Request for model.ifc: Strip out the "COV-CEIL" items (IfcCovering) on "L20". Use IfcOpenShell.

First a look at what the model holds.

```python
import ifcopenshell
import ifcopenshell.util.element

model = ifcopenshell.open("model.ifc")
print(model.schema)
storey = next(s for s in model.by_type("IfcBuildingStorey") if s.Name == "L20")
coverings = [e for e in ifcopenshell.util.element.get_decomposition(storey) if e.is_a("IfcCovering")]
seen = {}
for e in coverings:
    element_type = ifcopenshell.util.element.get_type(e)
    name = element_type.Name if element_type not in (None, e) else None
    seen[name] = seen.get(name, 0) + 1
for name, count in sorted(seen.items(), key=str):
    print(count, "x", name)
```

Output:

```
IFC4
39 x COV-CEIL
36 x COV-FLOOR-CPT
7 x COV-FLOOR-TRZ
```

```python
import ifcopenshell
import ifcopenshell.api.root
import ifcopenshell.util.element

model = ifcopenshell.open("model.ifc")

storey = next(s for s in model.by_type("IfcBuildingStorey") if s.Name == "L20")
coverings = [e for e in ifcopenshell.util.element.get_decomposition(storey) if e.is_a("IfcCovering")]
targets = [e for e in coverings if (t := ifcopenshell.util.element.get_type(e)) not in (None, e) and t.Name == "COV-CEIL"]

for e in targets:
    ifcopenshell.api.root.remove_product(model, product=e)
print(len(targets), "removed")

model.write("model_edited.ifc")
```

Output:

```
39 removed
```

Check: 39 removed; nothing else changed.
